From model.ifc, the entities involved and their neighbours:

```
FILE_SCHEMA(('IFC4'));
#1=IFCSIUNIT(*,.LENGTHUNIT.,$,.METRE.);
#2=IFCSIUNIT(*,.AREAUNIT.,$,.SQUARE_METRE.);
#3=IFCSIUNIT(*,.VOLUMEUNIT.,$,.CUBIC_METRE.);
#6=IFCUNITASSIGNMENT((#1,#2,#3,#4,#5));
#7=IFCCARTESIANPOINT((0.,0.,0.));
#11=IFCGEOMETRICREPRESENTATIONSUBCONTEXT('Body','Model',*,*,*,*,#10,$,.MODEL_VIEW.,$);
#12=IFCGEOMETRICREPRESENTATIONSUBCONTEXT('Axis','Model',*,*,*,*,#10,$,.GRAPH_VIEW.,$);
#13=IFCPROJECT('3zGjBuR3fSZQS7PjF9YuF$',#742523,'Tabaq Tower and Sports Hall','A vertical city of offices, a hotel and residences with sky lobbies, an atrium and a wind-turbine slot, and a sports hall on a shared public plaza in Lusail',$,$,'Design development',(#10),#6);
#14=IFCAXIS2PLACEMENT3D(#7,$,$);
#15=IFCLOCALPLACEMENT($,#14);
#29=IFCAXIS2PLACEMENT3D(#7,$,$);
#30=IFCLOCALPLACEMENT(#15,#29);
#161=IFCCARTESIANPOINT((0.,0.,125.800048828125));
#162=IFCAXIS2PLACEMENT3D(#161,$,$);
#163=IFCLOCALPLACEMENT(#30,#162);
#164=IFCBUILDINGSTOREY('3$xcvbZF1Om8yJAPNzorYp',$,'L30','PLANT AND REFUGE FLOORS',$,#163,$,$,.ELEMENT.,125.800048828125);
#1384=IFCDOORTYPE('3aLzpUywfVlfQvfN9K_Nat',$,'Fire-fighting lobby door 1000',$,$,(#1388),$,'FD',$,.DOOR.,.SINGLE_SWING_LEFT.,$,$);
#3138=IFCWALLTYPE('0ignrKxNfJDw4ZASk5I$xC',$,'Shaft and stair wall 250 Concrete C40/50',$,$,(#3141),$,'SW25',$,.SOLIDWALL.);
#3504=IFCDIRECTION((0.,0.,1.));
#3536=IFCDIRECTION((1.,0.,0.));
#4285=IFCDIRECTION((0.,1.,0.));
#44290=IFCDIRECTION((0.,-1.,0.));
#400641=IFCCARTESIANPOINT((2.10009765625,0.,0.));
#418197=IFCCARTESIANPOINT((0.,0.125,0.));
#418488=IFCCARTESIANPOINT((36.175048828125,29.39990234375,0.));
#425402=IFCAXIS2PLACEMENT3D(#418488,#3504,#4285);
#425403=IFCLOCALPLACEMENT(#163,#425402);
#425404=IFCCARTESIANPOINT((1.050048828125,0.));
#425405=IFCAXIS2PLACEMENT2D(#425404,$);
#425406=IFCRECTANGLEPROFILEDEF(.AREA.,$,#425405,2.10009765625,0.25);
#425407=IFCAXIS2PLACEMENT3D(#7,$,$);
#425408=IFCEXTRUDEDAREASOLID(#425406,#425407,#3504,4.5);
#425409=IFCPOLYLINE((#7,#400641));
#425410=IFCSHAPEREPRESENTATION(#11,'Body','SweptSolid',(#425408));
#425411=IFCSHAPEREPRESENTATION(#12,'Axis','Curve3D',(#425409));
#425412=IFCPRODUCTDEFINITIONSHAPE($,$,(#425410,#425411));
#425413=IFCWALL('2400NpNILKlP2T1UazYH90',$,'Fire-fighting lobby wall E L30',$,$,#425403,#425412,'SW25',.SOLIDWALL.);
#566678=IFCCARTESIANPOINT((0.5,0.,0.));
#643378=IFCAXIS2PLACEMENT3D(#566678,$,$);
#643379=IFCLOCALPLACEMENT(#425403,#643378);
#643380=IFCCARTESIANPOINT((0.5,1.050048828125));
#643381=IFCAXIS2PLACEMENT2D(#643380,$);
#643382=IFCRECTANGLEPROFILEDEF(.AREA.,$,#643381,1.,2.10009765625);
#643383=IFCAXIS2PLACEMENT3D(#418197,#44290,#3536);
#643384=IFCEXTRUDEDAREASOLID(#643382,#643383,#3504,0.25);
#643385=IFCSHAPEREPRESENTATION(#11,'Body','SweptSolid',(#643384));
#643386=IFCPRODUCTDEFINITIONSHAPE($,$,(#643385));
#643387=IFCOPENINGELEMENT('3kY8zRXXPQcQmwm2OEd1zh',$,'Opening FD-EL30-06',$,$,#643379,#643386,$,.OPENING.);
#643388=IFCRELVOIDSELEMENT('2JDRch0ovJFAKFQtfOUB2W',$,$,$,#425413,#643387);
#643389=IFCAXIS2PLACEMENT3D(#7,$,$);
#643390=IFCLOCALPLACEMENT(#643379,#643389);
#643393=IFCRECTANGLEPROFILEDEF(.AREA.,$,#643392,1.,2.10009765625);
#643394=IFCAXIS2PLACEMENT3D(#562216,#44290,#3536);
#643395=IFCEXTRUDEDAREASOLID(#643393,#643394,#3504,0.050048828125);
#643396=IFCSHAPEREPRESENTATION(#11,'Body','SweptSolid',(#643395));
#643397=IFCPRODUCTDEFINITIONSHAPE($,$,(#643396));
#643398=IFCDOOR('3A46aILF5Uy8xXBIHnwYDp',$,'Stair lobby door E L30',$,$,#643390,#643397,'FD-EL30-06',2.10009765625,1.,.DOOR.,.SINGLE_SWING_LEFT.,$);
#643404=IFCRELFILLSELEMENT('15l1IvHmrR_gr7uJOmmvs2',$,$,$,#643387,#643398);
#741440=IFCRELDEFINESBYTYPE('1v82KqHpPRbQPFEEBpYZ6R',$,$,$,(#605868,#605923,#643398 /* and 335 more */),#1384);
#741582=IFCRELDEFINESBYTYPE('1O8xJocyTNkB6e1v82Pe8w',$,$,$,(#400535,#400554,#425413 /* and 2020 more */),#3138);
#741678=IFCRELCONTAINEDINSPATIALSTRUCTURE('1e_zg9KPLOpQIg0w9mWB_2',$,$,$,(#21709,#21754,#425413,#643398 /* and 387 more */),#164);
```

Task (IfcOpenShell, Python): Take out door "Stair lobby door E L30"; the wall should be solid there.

```python
import ifcopenshell
import ifcopenshell.api.feature
import ifcopenshell.api.root
import ifcopenshell.geom
import ifcopenshell.util.shape

model = ifcopenshell.open("model.ifc")
settings = ifcopenshell.geom.settings()


def volume(element):
    """Net volume in cubic metres, openings subtracted."""
    shape = ifcopenshell.geom.create_shape(settings, element)
    return ifcopenshell.util.shape.get_volume(shape.geometry)


door = model.by_id(643398)
opening = door.FillsVoids[0].RelatingOpeningElement
wall = opening.VoidsElements[0].RelatingBuildingElement
before = volume(wall)

ifcopenshell.api.root.remove_product(model, product=door)
ifcopenshell.api.feature.remove_feature(model, feature=opening)

after = volume(wall)

print(f"wall volume {before:.3f} -> {after:.3f} m3")

model.write("model_v2.ifc")
```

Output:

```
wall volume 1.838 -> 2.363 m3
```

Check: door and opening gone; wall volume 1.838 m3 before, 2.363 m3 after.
